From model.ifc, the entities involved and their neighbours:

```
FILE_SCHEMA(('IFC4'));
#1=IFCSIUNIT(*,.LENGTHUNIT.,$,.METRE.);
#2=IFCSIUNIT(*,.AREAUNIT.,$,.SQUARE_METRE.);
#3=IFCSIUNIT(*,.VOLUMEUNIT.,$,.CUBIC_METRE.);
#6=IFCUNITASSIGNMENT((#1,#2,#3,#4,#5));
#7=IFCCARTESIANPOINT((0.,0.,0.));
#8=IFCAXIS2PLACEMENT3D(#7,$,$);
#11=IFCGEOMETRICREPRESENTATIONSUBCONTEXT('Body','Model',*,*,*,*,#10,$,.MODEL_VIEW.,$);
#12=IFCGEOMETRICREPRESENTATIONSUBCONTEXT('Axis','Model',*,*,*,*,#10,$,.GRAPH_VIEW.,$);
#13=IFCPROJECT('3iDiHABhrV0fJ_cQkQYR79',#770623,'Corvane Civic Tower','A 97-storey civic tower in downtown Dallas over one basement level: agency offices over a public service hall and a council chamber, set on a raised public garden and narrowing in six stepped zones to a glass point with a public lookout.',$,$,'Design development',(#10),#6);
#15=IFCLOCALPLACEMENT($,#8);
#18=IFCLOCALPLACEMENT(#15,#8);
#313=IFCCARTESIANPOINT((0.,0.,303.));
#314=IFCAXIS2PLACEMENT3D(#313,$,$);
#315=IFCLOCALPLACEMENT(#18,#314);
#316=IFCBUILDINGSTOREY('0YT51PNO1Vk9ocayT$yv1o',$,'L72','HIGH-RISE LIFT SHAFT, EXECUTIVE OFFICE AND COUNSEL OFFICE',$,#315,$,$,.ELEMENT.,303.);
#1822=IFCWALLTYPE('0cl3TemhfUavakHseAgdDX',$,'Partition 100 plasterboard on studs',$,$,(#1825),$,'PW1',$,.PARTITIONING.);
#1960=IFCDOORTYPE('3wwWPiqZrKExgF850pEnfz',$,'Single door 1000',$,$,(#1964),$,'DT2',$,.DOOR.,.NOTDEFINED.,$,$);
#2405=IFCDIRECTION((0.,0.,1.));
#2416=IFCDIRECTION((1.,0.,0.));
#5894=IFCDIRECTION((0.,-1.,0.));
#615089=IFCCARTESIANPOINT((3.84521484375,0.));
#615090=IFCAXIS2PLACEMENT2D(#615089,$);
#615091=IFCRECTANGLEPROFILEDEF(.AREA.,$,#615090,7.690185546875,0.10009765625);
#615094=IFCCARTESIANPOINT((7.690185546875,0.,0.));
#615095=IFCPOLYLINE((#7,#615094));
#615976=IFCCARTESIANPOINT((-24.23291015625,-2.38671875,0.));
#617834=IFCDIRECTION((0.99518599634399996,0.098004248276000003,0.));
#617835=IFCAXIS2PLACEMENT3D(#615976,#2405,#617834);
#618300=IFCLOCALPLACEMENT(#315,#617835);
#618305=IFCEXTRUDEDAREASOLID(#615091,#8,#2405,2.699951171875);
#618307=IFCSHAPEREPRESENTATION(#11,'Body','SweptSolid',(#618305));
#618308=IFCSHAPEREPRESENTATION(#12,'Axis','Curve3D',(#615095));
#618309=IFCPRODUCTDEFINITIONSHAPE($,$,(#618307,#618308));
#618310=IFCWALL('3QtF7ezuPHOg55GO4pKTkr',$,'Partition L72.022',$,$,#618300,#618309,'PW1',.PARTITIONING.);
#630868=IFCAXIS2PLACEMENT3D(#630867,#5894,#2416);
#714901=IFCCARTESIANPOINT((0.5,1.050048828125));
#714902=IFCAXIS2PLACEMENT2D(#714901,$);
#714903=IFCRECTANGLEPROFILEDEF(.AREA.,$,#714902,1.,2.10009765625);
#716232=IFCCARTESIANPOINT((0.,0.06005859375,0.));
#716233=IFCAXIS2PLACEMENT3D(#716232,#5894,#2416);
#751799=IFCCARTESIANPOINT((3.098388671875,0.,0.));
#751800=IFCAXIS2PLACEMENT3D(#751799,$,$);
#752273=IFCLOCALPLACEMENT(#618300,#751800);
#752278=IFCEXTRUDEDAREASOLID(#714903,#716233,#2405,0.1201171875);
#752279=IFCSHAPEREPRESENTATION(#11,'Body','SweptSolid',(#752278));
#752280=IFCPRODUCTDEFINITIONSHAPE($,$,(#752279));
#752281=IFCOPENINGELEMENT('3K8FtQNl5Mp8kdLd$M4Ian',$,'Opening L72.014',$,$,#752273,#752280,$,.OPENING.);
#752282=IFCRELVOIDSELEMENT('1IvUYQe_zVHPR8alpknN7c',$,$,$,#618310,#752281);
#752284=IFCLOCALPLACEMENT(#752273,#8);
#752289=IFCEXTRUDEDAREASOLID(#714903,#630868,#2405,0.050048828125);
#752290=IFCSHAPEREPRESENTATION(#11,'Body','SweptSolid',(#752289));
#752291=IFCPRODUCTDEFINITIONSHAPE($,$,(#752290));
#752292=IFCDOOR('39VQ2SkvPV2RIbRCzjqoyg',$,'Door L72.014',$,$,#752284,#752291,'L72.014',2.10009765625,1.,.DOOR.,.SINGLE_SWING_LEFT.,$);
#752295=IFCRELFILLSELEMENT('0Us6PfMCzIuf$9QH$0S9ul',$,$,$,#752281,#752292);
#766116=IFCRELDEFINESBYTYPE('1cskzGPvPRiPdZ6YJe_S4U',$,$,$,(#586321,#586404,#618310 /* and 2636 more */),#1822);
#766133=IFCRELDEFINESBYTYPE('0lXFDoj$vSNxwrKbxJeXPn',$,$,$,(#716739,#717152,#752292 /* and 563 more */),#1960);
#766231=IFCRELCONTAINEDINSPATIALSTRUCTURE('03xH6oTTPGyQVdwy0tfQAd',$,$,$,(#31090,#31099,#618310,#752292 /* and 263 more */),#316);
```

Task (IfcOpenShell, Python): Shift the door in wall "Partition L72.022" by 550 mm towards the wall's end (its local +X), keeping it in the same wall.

```python
import ifcopenshell
import ifcopenshell.api.geometry
import ifcopenshell.util.placement
import ifcopenshell.util.unit

model = ifcopenshell.open("model.ifc")
unit_scale = ifcopenshell.util.unit.calculate_unit_scale(model)

door = model.by_id(752292)
opening = door.FillsVoids[0].RelatingOpeningElement
wall = opening.VoidsElements[0].RelatingBuildingElement

wall_matrix = ifcopenshell.util.placement.get_local_placement(wall.ObjectPlacement)
shift = wall_matrix[:3, 0] * 0.55 / unit_scale
before = ifcopenshell.util.placement.get_local_placement(door.ObjectPlacement)[:3, 3].copy()

# The door is placed relative to its opening, so it follows when the opening moves.
matrix = ifcopenshell.util.placement.get_local_placement(opening.ObjectPlacement)
matrix[:3, 3] += shift
ifcopenshell.api.geometry.edit_object_placement(
    model, product=opening, matrix=matrix, is_si=False, should_transform_children=True
)

after = ifcopenshell.util.placement.get_local_placement(door.ObjectPlacement)[:3, 3]
print("door moved by", (after - before).round(3) + 0.0)

model.write("model-out.ifc")
```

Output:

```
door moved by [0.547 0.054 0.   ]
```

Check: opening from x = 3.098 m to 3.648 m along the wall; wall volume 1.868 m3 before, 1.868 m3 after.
